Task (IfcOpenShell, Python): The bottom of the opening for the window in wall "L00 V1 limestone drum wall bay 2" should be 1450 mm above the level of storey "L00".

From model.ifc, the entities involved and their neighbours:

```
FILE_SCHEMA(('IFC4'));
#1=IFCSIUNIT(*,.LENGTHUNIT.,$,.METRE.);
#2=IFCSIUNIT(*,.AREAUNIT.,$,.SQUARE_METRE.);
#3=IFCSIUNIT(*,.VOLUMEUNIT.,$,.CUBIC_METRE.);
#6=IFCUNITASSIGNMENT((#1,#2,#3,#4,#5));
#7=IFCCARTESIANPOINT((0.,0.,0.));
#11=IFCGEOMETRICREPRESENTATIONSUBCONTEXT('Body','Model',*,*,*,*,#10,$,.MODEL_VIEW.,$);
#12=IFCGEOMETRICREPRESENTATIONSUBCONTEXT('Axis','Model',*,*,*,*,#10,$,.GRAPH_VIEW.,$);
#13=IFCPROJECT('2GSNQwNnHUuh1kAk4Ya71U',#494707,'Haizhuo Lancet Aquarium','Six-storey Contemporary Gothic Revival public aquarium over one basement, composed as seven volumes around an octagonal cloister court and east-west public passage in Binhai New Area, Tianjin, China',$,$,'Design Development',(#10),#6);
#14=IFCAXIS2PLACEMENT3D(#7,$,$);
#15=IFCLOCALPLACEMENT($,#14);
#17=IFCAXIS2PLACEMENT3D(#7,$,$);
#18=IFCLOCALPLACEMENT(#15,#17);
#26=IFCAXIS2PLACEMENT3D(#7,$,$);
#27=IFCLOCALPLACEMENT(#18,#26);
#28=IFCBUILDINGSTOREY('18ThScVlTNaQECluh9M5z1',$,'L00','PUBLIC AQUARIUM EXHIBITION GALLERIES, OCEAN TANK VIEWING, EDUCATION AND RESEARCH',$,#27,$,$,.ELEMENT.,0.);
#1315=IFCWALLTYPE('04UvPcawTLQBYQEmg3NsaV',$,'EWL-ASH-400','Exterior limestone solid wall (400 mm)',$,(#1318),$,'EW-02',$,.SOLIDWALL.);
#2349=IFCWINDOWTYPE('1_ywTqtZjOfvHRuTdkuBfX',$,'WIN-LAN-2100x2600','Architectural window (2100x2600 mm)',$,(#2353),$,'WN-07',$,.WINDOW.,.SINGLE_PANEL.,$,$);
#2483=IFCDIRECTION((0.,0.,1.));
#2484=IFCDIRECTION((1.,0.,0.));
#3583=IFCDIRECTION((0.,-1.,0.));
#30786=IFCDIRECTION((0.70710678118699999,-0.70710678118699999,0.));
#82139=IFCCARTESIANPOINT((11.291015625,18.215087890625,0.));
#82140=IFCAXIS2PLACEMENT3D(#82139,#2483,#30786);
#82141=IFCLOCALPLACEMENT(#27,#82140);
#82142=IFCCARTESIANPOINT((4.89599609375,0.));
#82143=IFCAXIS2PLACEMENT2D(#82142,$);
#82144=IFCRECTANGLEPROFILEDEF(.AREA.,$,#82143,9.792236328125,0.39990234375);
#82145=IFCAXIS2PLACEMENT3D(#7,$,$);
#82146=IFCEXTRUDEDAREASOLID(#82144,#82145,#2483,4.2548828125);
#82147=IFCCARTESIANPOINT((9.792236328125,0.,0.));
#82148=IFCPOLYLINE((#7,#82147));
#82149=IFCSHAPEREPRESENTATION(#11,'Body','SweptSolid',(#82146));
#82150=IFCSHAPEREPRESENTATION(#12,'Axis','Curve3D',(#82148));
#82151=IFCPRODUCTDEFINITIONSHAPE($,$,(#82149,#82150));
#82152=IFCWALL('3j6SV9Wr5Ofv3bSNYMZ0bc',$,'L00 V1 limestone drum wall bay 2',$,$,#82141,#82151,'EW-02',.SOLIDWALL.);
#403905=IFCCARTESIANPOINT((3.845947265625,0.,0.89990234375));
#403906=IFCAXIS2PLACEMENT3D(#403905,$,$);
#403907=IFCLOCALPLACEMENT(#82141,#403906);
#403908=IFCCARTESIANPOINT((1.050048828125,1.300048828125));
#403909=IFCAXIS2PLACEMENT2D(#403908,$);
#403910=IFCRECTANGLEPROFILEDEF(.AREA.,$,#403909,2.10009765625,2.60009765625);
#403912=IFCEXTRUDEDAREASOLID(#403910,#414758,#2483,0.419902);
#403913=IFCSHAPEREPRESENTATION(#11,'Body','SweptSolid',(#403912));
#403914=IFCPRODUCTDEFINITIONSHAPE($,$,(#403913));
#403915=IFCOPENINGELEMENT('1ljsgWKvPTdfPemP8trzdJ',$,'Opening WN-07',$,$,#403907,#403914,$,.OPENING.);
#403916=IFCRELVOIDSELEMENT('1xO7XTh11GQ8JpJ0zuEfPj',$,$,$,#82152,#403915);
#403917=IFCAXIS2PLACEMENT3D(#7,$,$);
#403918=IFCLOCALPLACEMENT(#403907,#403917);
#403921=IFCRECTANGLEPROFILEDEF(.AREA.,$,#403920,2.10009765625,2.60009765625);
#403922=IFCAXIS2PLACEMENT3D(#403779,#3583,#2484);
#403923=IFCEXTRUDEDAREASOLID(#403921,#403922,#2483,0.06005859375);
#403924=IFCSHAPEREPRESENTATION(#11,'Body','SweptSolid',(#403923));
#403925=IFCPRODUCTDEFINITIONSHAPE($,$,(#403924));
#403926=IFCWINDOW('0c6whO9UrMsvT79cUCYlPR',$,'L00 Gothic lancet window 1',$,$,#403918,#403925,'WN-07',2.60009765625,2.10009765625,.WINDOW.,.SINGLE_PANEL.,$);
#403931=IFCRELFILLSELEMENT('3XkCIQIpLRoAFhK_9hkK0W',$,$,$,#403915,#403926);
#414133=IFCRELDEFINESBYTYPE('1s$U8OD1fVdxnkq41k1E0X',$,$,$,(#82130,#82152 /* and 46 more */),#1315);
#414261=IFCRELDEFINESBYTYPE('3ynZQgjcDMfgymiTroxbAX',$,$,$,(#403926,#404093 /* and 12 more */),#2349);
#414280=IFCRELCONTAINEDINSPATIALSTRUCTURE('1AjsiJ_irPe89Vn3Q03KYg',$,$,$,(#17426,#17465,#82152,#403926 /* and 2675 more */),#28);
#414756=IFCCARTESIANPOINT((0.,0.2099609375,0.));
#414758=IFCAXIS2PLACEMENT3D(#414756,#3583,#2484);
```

```python
import numpy as np
import ifcopenshell
import ifcopenshell.api.geometry
import ifcopenshell.geom
import ifcopenshell.util.element
import ifcopenshell.util.placement
import ifcopenshell.util.shape
import ifcopenshell.util.unit

model = ifcopenshell.open("model.ifc")
unit_scale = ifcopenshell.util.unit.calculate_unit_scale(model)

window = model.by_id(403926)
opening = window.FillsVoids[0].RelatingOpeningElement
storey = ifcopenshell.util.element.get_container(window, ifc_class="IfcBuildingStorey")
level = ifcopenshell.util.placement.get_local_placement(storey.ObjectPlacement)[2, 3]

# The opening's origin need not be at the sill, so measure its lowest point.
shape = ifcopenshell.geom.create_shape(ifcopenshell.geom.settings(), opening)
bottom = ifcopenshell.util.shape.get_shape_bottom_elevation(shape, shape.geometry) / unit_scale
dz = level + 1.45 / unit_scale - bottom

shift = np.array([0.0, 0.0, dz])
# The window is placed relative to its opening, so it follows when the opening moves.
matrix = ifcopenshell.util.placement.get_local_placement(opening.ObjectPlacement)
matrix[:3, 3] += shift
ifcopenshell.api.geometry.edit_object_placement(
    model, product=opening, matrix=matrix, is_si=False, should_transform_children=True
)

print(f"moved by {dz * unit_scale:+.3f} m")

model.write("model_updated.ifc")
```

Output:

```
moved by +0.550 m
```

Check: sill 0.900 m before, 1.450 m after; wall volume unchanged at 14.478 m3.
